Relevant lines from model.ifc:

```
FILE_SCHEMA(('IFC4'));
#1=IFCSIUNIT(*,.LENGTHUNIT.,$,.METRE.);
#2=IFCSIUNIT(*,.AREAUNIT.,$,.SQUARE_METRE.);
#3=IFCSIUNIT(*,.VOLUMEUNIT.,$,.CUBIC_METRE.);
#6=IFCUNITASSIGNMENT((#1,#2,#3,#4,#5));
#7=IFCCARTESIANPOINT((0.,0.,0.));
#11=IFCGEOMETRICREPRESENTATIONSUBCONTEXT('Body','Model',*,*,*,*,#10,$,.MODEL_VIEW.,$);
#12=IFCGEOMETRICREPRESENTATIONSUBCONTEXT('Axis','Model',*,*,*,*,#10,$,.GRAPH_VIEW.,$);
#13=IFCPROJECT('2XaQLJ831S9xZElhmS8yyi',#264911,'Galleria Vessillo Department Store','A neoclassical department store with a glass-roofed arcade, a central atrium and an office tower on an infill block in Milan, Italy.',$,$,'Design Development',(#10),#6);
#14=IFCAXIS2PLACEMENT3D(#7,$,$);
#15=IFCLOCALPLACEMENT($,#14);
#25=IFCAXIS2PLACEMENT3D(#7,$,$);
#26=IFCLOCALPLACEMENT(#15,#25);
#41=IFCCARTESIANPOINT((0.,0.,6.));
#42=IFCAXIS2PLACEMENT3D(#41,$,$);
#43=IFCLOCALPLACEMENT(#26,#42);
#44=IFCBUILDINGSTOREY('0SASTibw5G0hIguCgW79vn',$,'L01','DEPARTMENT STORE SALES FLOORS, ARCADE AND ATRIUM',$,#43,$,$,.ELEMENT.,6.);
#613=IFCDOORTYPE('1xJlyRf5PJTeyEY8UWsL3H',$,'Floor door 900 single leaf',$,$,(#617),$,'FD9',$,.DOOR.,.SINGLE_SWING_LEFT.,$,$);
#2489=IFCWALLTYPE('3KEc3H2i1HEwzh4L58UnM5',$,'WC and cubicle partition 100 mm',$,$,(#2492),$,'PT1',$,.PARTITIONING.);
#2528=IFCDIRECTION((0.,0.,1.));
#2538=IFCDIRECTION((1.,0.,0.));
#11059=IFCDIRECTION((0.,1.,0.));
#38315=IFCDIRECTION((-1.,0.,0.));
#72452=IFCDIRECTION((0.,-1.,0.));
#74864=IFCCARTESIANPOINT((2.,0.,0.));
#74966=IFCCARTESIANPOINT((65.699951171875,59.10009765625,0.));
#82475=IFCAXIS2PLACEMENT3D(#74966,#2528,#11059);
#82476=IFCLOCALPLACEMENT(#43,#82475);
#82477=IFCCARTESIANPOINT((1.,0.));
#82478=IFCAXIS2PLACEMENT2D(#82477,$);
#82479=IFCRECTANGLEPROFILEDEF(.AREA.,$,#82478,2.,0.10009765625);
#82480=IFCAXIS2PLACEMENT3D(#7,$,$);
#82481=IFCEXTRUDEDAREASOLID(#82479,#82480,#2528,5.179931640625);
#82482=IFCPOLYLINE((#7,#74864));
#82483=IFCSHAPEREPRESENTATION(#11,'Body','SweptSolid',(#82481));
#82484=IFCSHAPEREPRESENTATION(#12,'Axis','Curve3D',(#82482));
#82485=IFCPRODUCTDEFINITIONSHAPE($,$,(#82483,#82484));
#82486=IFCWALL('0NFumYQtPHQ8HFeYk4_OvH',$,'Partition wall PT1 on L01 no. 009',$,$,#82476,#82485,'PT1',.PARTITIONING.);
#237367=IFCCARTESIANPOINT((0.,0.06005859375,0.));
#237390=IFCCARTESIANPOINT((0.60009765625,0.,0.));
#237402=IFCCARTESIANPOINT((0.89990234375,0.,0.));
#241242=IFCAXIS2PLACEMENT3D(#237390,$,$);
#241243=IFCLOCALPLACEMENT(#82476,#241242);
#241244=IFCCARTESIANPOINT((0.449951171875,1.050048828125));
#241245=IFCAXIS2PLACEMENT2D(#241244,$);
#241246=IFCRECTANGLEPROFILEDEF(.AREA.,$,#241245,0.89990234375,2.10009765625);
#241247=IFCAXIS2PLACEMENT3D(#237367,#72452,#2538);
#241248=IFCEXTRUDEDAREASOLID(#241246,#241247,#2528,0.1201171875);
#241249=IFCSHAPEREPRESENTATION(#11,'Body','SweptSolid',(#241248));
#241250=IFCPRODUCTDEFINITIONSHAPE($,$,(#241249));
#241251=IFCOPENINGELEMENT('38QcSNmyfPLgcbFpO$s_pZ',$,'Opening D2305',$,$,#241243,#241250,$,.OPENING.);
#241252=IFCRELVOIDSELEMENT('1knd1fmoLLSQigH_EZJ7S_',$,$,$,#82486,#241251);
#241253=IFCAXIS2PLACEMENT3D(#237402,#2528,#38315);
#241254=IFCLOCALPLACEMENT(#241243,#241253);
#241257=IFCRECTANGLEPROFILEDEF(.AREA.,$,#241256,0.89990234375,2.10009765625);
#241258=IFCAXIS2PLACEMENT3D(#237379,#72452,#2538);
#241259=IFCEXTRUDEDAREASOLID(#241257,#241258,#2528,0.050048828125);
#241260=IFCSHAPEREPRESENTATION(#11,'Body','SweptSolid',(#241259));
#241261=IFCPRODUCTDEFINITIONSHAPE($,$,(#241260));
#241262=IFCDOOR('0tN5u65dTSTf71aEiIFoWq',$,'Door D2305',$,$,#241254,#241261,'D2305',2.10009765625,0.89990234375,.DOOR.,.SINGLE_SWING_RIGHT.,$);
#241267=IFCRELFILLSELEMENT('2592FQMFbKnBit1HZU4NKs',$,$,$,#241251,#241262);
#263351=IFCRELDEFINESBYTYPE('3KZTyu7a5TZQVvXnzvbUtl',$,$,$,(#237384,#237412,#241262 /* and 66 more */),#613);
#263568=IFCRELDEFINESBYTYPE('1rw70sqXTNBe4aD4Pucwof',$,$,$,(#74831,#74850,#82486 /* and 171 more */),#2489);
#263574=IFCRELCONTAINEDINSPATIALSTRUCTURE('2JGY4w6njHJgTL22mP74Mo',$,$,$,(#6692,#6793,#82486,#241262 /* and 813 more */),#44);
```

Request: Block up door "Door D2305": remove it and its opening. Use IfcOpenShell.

```python
import ifcopenshell
import ifcopenshell.api.feature
import ifcopenshell.api.root
import ifcopenshell.geom
import ifcopenshell.util.shape

model = ifcopenshell.open("model.ifc")
settings = ifcopenshell.geom.settings()


def volume(element):
    """Net volume in cubic metres, openings subtracted."""
    shape = ifcopenshell.geom.create_shape(settings, element)
    return ifcopenshell.util.shape.get_volume(shape.geometry)


door = model.by_guid("0tN5u65dTSTf71aEiIFoWq")
opening = door.FillsVoids[0].RelatingOpeningElement
wall = opening.VoidsElements[0].RelatingBuildingElement
before = volume(wall)

ifcopenshell.api.root.remove_product(model, product=door)
ifcopenshell.api.feature.remove_feature(model, feature=opening)

after = volume(wall)

print(f"wall volume {before:.3f} -> {after:.3f} m3")

model.write("model_edited.ifc")
```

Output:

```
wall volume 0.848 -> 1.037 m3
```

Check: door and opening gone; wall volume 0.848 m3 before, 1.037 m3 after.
